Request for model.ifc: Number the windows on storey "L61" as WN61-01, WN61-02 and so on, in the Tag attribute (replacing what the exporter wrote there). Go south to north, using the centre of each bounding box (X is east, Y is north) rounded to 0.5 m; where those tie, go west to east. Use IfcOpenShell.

First a look at what the model holds.

```python
import ifcopenshell
import ifcopenshell.util.element
import ifcopenshell.util.placement

model = ifcopenshell.open("model.ifc")
print(model.schema)
storey = next(s for s in model.by_type("IfcBuildingStorey") if s.Name == "L61")
windows = [e for e in ifcopenshell.util.element.get_decomposition(storey) if e.is_a("IfcWindow")]
for e in sorted(windows, key=lambda e: e.id()):
    origin = ifcopenshell.util.placement.get_local_placement(e.ObjectPlacement)[:3, 3]
    print(e.id(), e.Tag, e.Name, origin.round(2) + 0.0, sep=" | ")
```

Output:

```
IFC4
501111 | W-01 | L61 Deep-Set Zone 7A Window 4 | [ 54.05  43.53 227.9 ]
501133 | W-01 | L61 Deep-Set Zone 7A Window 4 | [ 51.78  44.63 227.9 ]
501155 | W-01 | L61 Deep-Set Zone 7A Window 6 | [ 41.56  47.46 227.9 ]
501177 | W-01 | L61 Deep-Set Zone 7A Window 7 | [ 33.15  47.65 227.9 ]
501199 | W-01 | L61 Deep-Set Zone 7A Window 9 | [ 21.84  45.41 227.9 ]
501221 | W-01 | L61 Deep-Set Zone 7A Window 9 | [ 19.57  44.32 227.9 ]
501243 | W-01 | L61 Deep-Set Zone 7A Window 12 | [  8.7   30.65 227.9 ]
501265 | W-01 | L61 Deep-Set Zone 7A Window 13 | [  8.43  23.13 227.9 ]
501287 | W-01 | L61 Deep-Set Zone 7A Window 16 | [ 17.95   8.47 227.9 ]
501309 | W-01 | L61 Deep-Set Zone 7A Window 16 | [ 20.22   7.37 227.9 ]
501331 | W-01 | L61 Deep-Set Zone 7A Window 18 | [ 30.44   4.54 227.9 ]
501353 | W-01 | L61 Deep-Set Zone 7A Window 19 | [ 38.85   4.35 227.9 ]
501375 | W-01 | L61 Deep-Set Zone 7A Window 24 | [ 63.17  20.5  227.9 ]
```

```python
import ifcopenshell
import ifcopenshell.geom
import ifcopenshell.util.element
import ifcopenshell.util.shape

model = ifcopenshell.open("model.ifc")
settings = ifcopenshell.geom.settings()
settings.set("use-world-coords", True)


def centre(element):
    shape = ifcopenshell.geom.create_shape(settings, element)
    return ifcopenshell.util.shape.get_bbox_centroid(shape.geometry)


storey = next(s for s in model.by_type("IfcBuildingStorey") if s.Name == "L61")
windows = [e for e in ifcopenshell.util.element.get_decomposition(storey) if e.is_a("IfcWindow")]

# Insertion points can sit at a corner or the storey origin, so sort by the geometry (in metres).
centres = {e: centre(e) for e in windows}
windows.sort(key=lambda e: (round(centres[e][1] / 0.5), centres[e][0]))

for i, e in enumerate(windows, start=1):
    number = f"WN61-{i:02d}"
    e.Tag = number
    print(e.id(), number)

model.write("model_rev.ifc")
```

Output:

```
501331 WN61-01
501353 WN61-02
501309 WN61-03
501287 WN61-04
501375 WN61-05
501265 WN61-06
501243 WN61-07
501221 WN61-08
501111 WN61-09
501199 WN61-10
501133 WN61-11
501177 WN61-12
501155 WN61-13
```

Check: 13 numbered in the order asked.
